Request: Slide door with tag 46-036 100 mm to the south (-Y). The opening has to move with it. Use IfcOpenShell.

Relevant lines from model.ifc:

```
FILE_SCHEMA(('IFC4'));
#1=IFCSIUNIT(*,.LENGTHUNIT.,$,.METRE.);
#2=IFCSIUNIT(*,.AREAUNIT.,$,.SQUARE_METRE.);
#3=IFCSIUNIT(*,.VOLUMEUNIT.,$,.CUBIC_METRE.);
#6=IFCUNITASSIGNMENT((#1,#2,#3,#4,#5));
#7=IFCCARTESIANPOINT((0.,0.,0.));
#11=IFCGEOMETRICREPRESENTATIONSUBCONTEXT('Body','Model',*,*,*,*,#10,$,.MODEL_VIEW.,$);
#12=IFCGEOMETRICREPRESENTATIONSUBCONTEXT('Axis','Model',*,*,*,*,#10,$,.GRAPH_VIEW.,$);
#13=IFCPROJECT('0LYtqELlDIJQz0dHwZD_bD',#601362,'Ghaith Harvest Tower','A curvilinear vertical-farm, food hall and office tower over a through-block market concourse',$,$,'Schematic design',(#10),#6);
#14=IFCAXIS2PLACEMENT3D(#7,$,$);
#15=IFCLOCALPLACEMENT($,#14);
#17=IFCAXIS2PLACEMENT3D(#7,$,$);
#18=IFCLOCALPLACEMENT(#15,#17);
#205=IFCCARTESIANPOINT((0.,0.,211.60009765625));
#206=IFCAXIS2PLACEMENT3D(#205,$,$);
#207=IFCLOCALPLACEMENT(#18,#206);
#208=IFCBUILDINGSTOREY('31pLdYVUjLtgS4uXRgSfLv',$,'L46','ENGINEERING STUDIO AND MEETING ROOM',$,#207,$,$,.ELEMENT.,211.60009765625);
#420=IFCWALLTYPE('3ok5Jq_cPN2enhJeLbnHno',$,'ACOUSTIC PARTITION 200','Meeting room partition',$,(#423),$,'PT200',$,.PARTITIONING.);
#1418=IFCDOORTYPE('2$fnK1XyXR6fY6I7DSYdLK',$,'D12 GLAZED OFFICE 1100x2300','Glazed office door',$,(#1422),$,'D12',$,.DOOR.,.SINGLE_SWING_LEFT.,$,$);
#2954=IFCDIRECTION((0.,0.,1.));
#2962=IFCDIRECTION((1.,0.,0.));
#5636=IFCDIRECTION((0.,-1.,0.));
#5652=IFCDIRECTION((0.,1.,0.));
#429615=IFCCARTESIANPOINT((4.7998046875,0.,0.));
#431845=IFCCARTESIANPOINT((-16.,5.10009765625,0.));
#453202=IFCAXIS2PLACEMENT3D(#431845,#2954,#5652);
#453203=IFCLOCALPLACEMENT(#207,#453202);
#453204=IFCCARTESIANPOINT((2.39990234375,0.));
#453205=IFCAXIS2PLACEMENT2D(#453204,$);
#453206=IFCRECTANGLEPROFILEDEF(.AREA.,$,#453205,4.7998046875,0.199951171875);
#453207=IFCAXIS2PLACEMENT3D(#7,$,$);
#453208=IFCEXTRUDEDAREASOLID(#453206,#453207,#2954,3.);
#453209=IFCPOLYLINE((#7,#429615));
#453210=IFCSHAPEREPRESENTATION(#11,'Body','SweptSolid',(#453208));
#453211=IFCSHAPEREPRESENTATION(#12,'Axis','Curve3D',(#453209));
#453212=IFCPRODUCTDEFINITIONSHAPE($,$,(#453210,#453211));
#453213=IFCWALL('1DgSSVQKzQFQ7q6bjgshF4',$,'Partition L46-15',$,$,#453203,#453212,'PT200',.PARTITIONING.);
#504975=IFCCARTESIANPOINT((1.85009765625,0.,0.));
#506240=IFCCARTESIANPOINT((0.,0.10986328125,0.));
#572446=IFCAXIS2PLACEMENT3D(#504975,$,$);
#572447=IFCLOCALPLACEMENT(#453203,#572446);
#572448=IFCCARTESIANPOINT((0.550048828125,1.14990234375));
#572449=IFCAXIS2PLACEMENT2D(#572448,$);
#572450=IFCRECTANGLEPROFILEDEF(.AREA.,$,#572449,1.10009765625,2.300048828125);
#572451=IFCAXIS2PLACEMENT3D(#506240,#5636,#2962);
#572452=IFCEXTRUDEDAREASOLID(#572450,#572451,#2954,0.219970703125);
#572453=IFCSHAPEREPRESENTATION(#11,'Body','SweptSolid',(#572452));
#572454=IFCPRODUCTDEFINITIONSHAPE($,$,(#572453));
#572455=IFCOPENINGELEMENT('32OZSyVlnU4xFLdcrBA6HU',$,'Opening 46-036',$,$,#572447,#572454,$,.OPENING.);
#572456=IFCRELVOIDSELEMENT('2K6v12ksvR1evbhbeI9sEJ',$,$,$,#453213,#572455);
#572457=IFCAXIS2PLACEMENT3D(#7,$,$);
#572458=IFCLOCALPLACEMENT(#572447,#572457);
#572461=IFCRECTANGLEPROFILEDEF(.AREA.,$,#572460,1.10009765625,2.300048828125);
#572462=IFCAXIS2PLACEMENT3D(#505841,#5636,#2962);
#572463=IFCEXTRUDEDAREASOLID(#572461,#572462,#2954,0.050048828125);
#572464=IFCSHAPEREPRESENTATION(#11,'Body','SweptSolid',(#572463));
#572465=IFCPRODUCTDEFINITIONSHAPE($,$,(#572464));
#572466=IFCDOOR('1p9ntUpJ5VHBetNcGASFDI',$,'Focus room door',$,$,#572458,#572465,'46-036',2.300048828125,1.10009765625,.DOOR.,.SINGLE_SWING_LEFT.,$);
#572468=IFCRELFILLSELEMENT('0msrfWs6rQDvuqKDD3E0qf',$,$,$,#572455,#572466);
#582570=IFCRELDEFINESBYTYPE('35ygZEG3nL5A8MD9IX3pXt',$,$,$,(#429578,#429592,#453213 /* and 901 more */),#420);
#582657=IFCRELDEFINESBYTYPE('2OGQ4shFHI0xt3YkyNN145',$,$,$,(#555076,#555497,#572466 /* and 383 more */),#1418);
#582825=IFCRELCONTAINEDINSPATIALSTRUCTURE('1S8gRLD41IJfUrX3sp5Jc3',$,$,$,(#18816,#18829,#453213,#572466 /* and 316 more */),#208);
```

```python
import ifcopenshell
import ifcopenshell.api.geometry
import ifcopenshell.util.placement
import ifcopenshell.util.unit

model = ifcopenshell.open("model.ifc")
unit_scale = ifcopenshell.util.unit.calculate_unit_scale(model)

door = model.by_guid("1p9ntUpJ5VHBetNcGASFDI")
opening = door.FillsVoids[0].RelatingOpeningElement
wall = opening.VoidsElements[0].RelatingBuildingElement

wall_matrix = ifcopenshell.util.placement.get_local_placement(wall.ObjectPlacement)
shift = wall_matrix[:3, 0] * -0.1 / unit_scale
before = ifcopenshell.util.placement.get_local_placement(door.ObjectPlacement)[:3, 3].copy()

# The door is placed relative to its opening, so it follows when the opening moves.
matrix = ifcopenshell.util.placement.get_local_placement(opening.ObjectPlacement)
matrix[:3, 3] += shift
ifcopenshell.api.geometry.edit_object_placement(
    model, product=opening, matrix=matrix, is_si=False, should_transform_children=True
)

after = ifcopenshell.util.placement.get_local_placement(door.ObjectPlacement)[:3, 3]
print("door moved by", (after - before).round(3) + 0.0)

model.write("model_rev.ifc")
```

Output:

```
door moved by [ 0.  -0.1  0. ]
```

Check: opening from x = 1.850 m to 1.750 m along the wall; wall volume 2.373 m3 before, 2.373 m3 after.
